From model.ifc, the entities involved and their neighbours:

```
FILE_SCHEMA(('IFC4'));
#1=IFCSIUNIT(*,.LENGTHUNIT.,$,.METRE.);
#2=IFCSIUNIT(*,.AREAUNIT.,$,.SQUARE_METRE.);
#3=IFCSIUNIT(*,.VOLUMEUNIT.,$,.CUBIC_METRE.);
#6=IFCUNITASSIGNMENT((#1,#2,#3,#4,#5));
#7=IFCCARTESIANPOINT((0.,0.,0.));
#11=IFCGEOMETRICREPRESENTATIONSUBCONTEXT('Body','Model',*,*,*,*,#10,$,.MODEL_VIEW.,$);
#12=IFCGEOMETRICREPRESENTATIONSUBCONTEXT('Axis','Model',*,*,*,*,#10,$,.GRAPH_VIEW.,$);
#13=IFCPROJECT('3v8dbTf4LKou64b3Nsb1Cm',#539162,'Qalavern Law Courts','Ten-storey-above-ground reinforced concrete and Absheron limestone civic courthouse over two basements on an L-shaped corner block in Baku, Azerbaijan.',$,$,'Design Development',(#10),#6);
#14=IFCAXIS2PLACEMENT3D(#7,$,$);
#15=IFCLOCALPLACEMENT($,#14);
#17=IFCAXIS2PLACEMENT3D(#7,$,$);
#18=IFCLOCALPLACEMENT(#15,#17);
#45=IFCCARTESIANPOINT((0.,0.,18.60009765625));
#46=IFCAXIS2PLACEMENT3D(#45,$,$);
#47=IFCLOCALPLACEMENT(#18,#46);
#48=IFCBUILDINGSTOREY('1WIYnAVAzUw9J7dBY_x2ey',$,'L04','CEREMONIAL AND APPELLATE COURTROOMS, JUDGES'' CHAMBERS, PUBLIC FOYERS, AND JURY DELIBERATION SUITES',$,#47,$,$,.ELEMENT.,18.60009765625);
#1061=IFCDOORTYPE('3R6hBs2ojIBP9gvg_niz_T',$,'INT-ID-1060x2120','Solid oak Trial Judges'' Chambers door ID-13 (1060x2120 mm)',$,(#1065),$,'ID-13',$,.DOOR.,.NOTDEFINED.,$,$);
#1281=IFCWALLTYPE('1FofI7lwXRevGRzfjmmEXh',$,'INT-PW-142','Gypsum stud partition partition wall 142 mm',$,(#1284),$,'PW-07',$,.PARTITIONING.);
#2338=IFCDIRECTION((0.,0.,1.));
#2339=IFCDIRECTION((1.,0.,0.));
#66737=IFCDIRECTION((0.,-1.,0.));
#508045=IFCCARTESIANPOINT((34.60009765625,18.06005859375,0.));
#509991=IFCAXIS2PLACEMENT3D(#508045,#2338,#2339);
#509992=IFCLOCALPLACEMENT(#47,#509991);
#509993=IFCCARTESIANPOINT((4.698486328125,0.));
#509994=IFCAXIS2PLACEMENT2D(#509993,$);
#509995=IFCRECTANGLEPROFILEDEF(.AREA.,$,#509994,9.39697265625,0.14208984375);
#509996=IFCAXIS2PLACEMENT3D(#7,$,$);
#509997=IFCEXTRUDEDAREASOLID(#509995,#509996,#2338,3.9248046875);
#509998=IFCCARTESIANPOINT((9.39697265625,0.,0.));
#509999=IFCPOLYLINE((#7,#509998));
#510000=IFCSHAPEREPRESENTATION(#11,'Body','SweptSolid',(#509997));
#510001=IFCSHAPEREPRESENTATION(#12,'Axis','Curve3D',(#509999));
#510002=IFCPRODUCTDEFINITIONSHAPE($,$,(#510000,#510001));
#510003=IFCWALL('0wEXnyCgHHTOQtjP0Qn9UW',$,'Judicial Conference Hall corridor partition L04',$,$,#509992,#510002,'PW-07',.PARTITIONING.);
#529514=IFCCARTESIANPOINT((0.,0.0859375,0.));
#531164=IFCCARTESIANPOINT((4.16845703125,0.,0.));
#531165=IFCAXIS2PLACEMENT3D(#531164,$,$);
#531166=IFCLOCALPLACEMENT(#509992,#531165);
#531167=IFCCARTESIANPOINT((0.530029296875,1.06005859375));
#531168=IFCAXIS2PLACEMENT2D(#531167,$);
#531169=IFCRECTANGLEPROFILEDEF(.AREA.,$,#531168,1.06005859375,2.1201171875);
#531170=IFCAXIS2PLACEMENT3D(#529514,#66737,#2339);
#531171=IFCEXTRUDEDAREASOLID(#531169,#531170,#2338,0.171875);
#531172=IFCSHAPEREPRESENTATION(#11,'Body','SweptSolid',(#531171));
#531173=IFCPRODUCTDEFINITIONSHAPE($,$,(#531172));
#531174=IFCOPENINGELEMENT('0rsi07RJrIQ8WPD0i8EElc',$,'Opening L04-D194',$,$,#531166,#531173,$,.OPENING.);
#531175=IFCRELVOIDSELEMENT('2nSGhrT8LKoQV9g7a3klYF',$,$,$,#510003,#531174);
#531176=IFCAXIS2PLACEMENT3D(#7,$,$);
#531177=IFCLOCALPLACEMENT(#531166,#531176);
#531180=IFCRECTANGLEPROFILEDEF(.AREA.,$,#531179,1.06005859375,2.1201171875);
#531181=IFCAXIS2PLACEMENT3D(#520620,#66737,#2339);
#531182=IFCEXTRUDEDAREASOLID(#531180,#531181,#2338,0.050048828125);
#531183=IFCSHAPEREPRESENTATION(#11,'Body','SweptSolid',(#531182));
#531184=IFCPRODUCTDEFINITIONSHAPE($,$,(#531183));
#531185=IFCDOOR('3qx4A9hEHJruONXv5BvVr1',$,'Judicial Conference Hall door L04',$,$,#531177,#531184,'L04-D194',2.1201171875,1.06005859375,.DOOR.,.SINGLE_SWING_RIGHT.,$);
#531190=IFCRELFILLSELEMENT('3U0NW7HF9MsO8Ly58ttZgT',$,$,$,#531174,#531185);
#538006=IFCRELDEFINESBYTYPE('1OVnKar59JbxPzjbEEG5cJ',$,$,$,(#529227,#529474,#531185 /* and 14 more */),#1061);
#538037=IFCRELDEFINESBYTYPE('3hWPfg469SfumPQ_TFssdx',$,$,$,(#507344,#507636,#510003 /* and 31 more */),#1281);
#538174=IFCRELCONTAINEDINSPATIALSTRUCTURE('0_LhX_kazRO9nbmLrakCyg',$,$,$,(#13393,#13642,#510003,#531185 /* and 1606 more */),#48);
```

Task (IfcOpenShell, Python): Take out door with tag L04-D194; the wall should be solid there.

```python
import ifcopenshell
import ifcopenshell.api.feature
import ifcopenshell.api.root
import ifcopenshell.geom
import ifcopenshell.util.shape

model = ifcopenshell.open("model.ifc")
settings = ifcopenshell.geom.settings()


def volume(element):
    """Net volume in cubic metres, openings subtracted."""
    shape = ifcopenshell.geom.create_shape(settings, element)
    return ifcopenshell.util.shape.get_volume(shape.geometry)


door = model.by_guid("3qx4A9hEHJruONXv5BvVr1")
opening = door.FillsVoids[0].RelatingOpeningElement
wall = opening.VoidsElements[0].RelatingBuildingElement
before = volume(wall)

ifcopenshell.api.root.remove_product(model, product=door)
ifcopenshell.api.feature.remove_feature(model, feature=opening)

after = volume(wall)

print(f"wall volume {before:.3f} -> {after:.3f} m3")

model.write("model_rev.ifc")
```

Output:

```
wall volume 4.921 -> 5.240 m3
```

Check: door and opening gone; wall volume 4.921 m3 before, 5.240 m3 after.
